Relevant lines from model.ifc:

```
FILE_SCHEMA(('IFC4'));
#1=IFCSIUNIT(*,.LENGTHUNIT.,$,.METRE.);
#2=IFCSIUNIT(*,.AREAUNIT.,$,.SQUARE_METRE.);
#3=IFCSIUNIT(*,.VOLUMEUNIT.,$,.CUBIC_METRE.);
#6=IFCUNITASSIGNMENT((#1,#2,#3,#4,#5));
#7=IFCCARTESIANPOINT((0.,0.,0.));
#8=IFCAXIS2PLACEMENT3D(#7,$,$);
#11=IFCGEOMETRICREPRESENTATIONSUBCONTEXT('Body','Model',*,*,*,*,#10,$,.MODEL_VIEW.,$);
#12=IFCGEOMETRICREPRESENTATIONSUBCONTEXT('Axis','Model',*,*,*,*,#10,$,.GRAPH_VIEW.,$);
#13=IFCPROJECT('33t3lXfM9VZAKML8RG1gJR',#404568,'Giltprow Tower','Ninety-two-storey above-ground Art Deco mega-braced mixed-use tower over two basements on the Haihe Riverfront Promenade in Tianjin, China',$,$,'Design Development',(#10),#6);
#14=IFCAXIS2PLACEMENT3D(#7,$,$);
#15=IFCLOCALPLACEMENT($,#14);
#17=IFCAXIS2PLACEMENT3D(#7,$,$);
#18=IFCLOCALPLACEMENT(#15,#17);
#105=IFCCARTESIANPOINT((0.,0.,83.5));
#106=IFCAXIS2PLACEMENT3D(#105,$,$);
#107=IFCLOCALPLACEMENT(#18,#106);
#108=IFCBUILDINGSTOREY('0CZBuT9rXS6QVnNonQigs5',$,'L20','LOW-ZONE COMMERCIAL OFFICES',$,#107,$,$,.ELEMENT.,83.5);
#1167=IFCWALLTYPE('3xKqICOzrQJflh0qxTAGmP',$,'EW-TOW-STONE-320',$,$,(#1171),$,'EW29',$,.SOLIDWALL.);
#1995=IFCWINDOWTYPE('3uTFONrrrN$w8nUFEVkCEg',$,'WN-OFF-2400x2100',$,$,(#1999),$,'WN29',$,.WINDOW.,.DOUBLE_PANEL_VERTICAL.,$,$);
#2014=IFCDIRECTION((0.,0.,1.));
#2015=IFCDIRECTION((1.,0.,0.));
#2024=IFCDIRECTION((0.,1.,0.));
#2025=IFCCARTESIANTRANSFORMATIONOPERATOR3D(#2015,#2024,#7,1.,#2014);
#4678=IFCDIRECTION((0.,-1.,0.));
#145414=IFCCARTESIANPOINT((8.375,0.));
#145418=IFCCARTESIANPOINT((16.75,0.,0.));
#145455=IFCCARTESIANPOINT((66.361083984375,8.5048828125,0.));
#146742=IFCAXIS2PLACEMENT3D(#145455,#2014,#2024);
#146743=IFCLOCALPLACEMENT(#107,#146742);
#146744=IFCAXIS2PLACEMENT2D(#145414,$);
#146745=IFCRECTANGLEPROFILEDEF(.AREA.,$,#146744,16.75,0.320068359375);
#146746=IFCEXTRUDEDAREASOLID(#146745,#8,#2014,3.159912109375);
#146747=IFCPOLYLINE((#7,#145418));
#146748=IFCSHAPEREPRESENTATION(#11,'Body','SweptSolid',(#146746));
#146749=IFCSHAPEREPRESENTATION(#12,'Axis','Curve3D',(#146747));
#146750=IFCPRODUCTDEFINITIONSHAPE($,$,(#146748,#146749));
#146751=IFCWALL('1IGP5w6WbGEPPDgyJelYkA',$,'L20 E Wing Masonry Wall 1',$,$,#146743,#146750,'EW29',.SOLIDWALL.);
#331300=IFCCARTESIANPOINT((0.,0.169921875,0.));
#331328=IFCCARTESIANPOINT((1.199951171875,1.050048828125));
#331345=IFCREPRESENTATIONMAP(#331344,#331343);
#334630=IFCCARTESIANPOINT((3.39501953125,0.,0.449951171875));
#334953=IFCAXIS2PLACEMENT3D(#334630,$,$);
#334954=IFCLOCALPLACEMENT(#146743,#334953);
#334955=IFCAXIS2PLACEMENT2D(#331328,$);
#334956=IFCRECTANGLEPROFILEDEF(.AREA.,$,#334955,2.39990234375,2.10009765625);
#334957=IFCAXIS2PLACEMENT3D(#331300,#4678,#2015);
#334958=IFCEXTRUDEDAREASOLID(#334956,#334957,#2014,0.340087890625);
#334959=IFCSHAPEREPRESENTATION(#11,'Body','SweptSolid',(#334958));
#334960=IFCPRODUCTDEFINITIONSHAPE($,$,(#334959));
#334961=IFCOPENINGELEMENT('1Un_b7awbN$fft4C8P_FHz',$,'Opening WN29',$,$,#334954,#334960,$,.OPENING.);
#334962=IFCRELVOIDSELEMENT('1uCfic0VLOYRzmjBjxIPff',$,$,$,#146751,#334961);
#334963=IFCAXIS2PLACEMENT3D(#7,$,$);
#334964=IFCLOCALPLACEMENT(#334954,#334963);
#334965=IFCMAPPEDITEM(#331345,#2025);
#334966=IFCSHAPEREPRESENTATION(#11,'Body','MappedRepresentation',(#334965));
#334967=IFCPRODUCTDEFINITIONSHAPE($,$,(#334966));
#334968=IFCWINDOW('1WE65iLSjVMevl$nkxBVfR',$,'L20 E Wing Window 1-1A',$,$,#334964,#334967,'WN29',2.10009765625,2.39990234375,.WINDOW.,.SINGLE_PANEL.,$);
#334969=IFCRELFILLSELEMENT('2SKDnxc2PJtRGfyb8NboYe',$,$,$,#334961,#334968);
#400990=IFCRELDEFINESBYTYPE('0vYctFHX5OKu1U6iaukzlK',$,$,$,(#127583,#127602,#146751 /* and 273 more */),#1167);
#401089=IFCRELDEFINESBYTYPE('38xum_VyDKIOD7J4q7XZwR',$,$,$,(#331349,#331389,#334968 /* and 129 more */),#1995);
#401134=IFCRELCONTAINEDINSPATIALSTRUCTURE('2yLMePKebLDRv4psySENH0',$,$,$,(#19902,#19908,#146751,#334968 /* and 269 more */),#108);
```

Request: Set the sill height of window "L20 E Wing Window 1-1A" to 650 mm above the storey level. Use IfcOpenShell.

```python
import numpy as np
import ifcopenshell
import ifcopenshell.api.geometry
import ifcopenshell.geom
import ifcopenshell.util.element
import ifcopenshell.util.placement
import ifcopenshell.util.shape
import ifcopenshell.util.unit

model = ifcopenshell.open("model.ifc")
unit_scale = ifcopenshell.util.unit.calculate_unit_scale(model)

window = model.by_guid("1WE65iLSjVMevl$nkxBVfR")
opening = window.FillsVoids[0].RelatingOpeningElement
storey = ifcopenshell.util.element.get_container(window, ifc_class="IfcBuildingStorey")
level = ifcopenshell.util.placement.get_local_placement(storey.ObjectPlacement)[2, 3]

# The opening's origin need not be at the sill, so measure its lowest point.
shape = ifcopenshell.geom.create_shape(ifcopenshell.geom.settings(), opening)
bottom = ifcopenshell.util.shape.get_shape_bottom_elevation(shape, shape.geometry) / unit_scale
dz = level + 0.65 / unit_scale - bottom

shift = np.array([0.0, 0.0, dz])
# The window is placed relative to its opening, so it follows when the opening moves.
matrix = ifcopenshell.util.placement.get_local_placement(opening.ObjectPlacement)
matrix[:3, 3] += shift
ifcopenshell.api.geometry.edit_object_placement(
    model, product=opening, matrix=matrix, is_si=False, should_transform_children=True
)

print(f"moved by {dz * unit_scale:+.3f} m")

model.write("model-out.ifc")
```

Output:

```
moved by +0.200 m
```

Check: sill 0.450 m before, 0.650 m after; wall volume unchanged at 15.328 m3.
